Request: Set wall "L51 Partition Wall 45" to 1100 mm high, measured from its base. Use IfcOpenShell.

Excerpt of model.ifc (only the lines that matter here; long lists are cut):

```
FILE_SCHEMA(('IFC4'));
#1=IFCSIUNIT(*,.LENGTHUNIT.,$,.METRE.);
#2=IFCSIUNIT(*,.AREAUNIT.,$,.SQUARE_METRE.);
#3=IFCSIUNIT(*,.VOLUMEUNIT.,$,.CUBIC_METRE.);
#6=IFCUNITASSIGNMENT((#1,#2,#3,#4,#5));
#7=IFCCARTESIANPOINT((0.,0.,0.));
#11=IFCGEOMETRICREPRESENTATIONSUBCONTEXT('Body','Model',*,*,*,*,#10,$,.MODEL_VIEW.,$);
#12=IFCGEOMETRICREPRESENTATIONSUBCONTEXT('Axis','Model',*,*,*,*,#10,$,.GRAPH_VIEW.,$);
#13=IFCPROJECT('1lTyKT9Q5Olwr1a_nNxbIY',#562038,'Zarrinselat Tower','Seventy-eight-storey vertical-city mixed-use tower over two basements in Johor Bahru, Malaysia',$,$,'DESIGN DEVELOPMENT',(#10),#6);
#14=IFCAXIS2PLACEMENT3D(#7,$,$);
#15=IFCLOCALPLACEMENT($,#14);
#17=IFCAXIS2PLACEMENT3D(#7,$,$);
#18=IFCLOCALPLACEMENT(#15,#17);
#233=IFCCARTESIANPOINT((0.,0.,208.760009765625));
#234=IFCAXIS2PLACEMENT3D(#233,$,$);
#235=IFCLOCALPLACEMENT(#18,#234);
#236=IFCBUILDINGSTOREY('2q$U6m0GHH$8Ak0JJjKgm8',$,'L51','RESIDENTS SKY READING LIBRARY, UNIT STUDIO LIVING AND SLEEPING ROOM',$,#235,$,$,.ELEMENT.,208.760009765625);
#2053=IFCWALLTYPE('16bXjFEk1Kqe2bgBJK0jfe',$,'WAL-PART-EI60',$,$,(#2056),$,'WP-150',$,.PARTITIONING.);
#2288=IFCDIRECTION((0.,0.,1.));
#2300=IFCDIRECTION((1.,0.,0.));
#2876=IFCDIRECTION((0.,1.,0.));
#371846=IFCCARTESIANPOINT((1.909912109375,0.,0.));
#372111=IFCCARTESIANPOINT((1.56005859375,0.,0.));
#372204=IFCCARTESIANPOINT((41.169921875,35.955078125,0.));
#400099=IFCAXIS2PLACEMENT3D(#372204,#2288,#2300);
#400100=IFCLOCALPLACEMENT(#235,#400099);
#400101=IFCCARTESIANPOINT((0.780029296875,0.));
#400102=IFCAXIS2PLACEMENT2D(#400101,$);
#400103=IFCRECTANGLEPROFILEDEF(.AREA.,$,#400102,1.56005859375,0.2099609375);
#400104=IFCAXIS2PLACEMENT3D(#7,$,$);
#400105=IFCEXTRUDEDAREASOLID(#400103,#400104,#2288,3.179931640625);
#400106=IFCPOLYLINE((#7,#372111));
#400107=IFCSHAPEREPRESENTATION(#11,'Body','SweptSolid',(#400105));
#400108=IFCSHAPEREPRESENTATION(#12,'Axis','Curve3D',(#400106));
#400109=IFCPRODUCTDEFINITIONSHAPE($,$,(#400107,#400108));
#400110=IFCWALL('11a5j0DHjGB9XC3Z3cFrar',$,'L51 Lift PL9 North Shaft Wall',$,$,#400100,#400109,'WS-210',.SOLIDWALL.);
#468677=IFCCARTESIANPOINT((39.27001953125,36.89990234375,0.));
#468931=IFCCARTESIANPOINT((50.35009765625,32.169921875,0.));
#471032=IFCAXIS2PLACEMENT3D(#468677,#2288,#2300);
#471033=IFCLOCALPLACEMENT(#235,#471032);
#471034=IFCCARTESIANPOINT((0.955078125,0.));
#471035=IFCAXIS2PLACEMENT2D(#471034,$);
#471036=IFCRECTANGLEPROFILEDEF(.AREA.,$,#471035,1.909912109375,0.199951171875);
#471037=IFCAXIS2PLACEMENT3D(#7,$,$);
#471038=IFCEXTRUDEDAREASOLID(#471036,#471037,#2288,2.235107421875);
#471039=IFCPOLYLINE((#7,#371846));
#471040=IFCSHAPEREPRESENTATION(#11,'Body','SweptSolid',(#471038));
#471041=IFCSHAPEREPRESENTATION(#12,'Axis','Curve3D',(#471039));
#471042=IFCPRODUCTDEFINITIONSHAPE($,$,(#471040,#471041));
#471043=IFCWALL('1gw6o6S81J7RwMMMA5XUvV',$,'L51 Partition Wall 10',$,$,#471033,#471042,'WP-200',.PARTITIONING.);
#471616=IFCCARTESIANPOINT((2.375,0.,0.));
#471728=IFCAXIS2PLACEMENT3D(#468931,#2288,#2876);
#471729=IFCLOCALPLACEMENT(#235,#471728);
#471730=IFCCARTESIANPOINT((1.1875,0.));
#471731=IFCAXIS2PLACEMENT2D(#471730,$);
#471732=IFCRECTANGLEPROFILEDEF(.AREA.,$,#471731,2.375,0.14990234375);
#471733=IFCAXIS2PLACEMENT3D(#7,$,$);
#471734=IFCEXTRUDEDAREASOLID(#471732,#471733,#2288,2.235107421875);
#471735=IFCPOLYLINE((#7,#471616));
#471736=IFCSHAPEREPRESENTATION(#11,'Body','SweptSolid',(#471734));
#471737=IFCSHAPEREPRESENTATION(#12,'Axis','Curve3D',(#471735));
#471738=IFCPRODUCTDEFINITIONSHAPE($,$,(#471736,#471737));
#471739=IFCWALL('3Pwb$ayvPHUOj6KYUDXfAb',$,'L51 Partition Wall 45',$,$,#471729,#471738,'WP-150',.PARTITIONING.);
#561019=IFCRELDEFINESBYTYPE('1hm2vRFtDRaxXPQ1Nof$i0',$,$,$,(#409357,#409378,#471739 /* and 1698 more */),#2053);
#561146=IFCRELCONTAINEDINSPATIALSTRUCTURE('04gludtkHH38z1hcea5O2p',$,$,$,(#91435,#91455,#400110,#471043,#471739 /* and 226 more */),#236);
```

```python
import ifcopenshell
import ifcopenshell.geom
import ifcopenshell.util.representation
import ifcopenshell.util.shape
import ifcopenshell.util.unit

model = ifcopenshell.open("model.ifc")
unit_scale = ifcopenshell.util.unit.calculate_unit_scale(model)
settings = ifcopenshell.geom.settings()


def volume(element):
    """Net volume in cubic metres, openings subtracted."""
    shape = ifcopenshell.geom.create_shape(settings, element)
    return ifcopenshell.util.shape.get_volume(shape.geometry)


wall = model.by_guid("3Pwb$ayvPHUOj6KYUDXfAb")
before = volume(wall)

body = ifcopenshell.util.representation.get_representation(wall, "Model", "Body")
solid = body.Items[0]
old_height = solid.Depth
solid.Depth = 1.1 / unit_scale
after = volume(wall)

print(f"height {old_height:g} -> {solid.Depth:g}, volume {before:.3f} -> {after:.3f} m3")

model.write("model_v2.ifc")
```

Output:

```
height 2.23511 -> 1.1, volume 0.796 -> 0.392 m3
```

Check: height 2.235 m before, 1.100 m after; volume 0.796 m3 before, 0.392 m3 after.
